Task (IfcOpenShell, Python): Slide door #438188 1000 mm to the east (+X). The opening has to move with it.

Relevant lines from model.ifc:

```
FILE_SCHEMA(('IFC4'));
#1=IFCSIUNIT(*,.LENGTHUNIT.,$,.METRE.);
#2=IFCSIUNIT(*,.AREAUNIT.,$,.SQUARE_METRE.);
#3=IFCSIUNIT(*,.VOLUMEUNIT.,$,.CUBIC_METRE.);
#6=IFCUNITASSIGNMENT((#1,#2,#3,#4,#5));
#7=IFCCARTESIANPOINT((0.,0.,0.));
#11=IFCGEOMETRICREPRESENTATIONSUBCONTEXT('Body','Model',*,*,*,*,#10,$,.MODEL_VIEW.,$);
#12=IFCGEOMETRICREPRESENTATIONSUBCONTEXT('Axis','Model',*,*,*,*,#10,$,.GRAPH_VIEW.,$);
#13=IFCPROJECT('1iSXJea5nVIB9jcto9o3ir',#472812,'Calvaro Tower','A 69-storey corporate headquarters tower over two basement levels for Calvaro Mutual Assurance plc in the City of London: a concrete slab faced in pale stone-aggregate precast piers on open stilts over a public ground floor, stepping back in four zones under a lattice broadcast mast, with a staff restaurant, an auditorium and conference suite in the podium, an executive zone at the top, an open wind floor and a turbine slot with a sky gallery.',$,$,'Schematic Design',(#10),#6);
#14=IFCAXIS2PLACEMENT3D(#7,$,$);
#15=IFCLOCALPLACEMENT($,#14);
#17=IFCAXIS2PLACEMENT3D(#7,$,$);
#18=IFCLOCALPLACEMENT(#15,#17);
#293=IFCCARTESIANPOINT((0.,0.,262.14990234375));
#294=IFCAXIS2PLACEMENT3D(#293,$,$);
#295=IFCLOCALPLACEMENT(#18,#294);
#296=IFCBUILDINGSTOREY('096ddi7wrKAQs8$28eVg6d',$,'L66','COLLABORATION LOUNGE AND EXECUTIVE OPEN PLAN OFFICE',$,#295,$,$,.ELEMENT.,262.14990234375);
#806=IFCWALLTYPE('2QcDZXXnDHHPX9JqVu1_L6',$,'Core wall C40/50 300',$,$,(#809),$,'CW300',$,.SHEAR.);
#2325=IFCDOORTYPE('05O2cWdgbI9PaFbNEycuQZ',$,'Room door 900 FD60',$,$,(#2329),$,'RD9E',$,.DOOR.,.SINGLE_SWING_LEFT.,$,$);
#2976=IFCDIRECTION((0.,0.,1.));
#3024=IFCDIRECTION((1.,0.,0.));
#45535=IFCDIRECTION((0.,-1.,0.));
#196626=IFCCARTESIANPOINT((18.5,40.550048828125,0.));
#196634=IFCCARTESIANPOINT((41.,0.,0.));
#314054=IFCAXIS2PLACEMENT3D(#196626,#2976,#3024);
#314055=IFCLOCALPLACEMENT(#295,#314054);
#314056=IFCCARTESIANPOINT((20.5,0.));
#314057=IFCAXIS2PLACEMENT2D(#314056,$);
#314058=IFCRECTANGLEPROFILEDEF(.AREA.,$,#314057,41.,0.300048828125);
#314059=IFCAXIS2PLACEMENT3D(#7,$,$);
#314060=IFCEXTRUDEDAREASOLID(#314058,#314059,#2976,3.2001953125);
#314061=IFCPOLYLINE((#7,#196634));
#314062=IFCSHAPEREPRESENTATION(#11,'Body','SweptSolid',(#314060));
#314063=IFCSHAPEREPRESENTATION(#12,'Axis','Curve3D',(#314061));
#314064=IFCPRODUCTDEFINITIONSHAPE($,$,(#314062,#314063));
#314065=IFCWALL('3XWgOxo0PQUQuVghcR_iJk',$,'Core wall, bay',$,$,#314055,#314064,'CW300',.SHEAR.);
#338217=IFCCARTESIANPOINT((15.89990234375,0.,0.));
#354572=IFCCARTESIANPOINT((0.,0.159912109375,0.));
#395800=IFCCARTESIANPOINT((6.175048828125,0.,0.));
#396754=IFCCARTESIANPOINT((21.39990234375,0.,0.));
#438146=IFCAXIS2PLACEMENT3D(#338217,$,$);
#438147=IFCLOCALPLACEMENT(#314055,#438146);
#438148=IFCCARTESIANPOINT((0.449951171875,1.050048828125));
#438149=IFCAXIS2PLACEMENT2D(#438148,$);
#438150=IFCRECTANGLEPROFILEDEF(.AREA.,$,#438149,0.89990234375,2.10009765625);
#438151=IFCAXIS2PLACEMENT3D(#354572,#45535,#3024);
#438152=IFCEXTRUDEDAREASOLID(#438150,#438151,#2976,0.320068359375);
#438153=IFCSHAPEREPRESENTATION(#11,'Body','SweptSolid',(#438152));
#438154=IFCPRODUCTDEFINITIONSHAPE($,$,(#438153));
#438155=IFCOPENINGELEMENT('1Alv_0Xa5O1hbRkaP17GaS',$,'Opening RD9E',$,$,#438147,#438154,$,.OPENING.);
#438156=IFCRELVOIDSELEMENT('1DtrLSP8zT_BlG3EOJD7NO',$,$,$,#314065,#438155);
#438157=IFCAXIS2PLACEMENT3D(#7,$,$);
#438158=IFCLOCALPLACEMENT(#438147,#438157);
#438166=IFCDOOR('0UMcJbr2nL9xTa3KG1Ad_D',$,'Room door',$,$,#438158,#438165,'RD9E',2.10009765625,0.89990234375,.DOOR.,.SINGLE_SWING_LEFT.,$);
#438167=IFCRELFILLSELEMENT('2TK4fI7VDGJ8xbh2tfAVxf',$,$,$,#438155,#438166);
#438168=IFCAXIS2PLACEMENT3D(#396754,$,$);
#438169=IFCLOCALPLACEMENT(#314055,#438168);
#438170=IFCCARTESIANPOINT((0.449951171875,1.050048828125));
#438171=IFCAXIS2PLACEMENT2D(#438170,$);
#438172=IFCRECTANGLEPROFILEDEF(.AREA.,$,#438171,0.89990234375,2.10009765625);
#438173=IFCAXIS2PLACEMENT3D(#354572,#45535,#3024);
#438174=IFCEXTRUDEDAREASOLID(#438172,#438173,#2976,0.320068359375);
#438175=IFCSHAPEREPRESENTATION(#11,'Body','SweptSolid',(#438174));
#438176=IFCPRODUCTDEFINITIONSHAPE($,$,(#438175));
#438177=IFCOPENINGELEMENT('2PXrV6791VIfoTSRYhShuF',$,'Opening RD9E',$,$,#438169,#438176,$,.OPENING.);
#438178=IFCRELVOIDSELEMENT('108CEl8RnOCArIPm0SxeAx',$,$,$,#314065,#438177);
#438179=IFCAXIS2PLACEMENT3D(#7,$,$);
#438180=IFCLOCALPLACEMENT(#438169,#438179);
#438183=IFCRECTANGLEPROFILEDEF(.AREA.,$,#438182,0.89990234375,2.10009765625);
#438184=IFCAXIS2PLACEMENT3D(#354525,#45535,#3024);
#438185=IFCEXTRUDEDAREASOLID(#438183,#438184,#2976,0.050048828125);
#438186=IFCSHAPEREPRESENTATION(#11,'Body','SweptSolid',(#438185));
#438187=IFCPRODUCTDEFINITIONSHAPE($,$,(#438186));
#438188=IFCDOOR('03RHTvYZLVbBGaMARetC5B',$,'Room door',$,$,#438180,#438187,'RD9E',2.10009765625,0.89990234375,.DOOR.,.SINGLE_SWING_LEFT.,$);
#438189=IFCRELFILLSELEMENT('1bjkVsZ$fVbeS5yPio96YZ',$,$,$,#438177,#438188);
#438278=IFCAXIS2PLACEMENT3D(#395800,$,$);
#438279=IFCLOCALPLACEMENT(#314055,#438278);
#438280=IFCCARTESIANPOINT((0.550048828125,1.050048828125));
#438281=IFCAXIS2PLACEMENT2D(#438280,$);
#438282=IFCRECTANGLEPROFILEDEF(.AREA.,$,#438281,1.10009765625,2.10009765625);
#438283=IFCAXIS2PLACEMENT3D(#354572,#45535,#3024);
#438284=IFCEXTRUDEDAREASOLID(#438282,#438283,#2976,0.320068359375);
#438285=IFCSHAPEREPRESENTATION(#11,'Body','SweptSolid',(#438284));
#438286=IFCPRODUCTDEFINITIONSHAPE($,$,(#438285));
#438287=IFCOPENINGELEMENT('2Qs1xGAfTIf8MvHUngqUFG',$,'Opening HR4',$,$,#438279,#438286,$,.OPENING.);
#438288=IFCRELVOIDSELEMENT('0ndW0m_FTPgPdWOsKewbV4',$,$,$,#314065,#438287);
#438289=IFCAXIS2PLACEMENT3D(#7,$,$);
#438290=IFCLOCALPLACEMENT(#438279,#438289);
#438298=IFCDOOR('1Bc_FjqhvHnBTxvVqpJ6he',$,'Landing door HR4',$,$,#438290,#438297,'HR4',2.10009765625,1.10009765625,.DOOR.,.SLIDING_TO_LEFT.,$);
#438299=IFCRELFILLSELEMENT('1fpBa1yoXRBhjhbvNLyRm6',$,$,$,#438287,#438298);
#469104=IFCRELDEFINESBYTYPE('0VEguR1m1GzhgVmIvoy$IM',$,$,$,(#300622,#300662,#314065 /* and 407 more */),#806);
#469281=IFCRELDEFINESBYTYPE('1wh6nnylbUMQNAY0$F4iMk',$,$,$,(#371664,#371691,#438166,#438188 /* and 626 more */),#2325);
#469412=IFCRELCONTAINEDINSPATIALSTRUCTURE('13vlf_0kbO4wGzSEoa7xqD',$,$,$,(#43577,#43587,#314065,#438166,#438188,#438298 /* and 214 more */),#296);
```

```python
import ifcopenshell
import ifcopenshell.api.geometry
import ifcopenshell.util.placement
import ifcopenshell.util.unit

model = ifcopenshell.open("model.ifc")
unit_scale = ifcopenshell.util.unit.calculate_unit_scale(model)

door = model.by_guid("03RHTvYZLVbBGaMARetC5B")
opening = door.FillsVoids[0].RelatingOpeningElement
wall = opening.VoidsElements[0].RelatingBuildingElement

wall_matrix = ifcopenshell.util.placement.get_local_placement(wall.ObjectPlacement)
shift = wall_matrix[:3, 0] * 1 / unit_scale
before = ifcopenshell.util.placement.get_local_placement(door.ObjectPlacement)[:3, 3].copy()

# The door is placed relative to its opening, so it follows when the opening moves.
matrix = ifcopenshell.util.placement.get_local_placement(opening.ObjectPlacement)
matrix[:3, 3] += shift
ifcopenshell.api.geometry.edit_object_placement(
    model, product=opening, matrix=matrix, is_si=False, should_transform_children=True
)

after = ifcopenshell.util.placement.get_local_placement(door.ObjectPlacement)[:3, 3]
print("door moved by", (after - before).round(3) + 0.0)

model.write("model_updated.ifc")
```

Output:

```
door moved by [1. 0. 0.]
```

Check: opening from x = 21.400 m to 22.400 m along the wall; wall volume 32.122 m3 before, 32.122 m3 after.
